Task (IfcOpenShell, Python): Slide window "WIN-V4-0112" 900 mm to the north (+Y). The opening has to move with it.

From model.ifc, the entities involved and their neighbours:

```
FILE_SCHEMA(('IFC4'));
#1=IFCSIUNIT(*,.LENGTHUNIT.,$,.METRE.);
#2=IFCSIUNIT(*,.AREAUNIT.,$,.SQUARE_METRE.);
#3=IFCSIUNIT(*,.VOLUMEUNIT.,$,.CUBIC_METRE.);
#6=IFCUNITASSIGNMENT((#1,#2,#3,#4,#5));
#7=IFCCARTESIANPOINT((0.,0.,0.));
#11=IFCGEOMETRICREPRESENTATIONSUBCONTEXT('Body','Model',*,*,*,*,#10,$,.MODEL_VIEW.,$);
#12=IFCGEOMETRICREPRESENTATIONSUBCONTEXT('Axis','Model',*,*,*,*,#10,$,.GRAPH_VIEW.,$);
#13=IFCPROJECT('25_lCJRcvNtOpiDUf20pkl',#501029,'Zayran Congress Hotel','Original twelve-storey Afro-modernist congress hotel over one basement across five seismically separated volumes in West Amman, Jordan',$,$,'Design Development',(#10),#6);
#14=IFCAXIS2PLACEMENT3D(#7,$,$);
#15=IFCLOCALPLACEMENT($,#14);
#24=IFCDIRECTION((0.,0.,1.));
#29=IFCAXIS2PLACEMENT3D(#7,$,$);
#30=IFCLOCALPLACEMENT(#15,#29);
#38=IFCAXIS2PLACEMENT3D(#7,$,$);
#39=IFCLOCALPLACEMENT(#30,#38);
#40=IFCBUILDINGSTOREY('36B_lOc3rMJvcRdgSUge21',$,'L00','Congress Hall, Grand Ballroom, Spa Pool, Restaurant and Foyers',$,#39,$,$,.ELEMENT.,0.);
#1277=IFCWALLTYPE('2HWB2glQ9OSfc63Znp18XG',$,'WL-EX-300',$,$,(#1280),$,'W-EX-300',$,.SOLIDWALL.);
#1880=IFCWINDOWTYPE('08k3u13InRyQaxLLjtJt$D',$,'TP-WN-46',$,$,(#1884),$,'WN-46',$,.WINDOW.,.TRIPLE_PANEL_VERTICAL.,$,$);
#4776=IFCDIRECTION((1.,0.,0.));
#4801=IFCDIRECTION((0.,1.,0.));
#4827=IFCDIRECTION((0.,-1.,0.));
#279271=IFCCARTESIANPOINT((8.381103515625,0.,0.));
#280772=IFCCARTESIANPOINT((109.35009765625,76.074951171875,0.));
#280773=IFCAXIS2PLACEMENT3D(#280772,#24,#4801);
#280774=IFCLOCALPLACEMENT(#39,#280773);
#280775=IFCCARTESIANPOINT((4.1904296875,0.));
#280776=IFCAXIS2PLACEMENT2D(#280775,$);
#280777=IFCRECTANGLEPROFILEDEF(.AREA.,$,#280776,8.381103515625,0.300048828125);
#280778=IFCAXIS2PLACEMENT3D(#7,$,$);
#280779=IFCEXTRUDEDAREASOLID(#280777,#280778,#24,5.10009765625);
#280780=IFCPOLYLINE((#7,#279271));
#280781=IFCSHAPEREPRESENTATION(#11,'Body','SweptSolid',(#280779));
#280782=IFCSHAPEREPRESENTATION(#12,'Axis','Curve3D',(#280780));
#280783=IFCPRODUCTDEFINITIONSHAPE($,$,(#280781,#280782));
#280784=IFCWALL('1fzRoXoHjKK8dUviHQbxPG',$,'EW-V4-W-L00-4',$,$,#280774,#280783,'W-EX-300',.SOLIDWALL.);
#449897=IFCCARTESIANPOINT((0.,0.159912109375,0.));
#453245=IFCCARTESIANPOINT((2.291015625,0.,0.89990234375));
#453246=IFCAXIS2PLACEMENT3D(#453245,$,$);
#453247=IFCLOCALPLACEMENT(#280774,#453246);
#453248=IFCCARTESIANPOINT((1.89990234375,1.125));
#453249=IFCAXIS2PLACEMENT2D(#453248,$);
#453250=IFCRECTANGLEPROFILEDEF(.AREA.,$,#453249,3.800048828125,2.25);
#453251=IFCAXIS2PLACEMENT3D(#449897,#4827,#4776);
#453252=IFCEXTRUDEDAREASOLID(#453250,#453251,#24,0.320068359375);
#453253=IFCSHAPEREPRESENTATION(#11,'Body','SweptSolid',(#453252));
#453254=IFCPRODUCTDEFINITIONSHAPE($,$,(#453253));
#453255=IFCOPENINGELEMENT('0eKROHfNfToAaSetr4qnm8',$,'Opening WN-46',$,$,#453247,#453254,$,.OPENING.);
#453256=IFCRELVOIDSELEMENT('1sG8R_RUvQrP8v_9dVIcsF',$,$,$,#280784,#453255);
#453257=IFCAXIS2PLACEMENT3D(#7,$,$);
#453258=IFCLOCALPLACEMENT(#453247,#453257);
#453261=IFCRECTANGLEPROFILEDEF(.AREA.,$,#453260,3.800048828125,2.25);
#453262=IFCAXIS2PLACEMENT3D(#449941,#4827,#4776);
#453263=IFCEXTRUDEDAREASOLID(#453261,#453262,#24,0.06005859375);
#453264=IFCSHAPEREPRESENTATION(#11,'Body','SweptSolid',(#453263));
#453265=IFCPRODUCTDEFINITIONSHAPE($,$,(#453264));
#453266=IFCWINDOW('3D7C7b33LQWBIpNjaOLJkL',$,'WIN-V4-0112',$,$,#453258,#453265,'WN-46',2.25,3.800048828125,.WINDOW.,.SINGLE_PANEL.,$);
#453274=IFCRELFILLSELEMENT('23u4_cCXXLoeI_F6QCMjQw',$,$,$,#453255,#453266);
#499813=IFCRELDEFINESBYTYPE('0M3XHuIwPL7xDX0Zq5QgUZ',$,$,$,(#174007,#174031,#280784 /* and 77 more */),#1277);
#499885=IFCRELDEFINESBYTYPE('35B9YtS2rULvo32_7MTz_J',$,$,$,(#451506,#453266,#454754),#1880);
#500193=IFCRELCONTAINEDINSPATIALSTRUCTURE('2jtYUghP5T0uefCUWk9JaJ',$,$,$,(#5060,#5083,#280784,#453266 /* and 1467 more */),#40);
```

```python
import ifcopenshell
import ifcopenshell.api.geometry
import ifcopenshell.util.placement
import ifcopenshell.util.unit

model = ifcopenshell.open("model.ifc")
unit_scale = ifcopenshell.util.unit.calculate_unit_scale(model)

window = model.by_guid("3D7C7b33LQWBIpNjaOLJkL")
opening = window.FillsVoids[0].RelatingOpeningElement
wall = opening.VoidsElements[0].RelatingBuildingElement

wall_matrix = ifcopenshell.util.placement.get_local_placement(wall.ObjectPlacement)
shift = wall_matrix[:3, 0] * 0.9 / unit_scale
before = ifcopenshell.util.placement.get_local_placement(window.ObjectPlacement)[:3, 3].copy()

# The window is placed relative to its opening, so it follows when the opening moves.
matrix = ifcopenshell.util.placement.get_local_placement(opening.ObjectPlacement)
matrix[:3, 3] += shift
ifcopenshell.api.geometry.edit_object_placement(
    model, product=opening, matrix=matrix, is_si=False, should_transform_children=True
)

after = ifcopenshell.util.placement.get_local_placement(window.ObjectPlacement)[:3, 3]
print("window moved by", (after - before).round(3) + 0.0)

model.write("model_rev.ifc")
```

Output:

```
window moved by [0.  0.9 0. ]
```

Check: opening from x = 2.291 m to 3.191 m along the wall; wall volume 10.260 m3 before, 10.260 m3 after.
